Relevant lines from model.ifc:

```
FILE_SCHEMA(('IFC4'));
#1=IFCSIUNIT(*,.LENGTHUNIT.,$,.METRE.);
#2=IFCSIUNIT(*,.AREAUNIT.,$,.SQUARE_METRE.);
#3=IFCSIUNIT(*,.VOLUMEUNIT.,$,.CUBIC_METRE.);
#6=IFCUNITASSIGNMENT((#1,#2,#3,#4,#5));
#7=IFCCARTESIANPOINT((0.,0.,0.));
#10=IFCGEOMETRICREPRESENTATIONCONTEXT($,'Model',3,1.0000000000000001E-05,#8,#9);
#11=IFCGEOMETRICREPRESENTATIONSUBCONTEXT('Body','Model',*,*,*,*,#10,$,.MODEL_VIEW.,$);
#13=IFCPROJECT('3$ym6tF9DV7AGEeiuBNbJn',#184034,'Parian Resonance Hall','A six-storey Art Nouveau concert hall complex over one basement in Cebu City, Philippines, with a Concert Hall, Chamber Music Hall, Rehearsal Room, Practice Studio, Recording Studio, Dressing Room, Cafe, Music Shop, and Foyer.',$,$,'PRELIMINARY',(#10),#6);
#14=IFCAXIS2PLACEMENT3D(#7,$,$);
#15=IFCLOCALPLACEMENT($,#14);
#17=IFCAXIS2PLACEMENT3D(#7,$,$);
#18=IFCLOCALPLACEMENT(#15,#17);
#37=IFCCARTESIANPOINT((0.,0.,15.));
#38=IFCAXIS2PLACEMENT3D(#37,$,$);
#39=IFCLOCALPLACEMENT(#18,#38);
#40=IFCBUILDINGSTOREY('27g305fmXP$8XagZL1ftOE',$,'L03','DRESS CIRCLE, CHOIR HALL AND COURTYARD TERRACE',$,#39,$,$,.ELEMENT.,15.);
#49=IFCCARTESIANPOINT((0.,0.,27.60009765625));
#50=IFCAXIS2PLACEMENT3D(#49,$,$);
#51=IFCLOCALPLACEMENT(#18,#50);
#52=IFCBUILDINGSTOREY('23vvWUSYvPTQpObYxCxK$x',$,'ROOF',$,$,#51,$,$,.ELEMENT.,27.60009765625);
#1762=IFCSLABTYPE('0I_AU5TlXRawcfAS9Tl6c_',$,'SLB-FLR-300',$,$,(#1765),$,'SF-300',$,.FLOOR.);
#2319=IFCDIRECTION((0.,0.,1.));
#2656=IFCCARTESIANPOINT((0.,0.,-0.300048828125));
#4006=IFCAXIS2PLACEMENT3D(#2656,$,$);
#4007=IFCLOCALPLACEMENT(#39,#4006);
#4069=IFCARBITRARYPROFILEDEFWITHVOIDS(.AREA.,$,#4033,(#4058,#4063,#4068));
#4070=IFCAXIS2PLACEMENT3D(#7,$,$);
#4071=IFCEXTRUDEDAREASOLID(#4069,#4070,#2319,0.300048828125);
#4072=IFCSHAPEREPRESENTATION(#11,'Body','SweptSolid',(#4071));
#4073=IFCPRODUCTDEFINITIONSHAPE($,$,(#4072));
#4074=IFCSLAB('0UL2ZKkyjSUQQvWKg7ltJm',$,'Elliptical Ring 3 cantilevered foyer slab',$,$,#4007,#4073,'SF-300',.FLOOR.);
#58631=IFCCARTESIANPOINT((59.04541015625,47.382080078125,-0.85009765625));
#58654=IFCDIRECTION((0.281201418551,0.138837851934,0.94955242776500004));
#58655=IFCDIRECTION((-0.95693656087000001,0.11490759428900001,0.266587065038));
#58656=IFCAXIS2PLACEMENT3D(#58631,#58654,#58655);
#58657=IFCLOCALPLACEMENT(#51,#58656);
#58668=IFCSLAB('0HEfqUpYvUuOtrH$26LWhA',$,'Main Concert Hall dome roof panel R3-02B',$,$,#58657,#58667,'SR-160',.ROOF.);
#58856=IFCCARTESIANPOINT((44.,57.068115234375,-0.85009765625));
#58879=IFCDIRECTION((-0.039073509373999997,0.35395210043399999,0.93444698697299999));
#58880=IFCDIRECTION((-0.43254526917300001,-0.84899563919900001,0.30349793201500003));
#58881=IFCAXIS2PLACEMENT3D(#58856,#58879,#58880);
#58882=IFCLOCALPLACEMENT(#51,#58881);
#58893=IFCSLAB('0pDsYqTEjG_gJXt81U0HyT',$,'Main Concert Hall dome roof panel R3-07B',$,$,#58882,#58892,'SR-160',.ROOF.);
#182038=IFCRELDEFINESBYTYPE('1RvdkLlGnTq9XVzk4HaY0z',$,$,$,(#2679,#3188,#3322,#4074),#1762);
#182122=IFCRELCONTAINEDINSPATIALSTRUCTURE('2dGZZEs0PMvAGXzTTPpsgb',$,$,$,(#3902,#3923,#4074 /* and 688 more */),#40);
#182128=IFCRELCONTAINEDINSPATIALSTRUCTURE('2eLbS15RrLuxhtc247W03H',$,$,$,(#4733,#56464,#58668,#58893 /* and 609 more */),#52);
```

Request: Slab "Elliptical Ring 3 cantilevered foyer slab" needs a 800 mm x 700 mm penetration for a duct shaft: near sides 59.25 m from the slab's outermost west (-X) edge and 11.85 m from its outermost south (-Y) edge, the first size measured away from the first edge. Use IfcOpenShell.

```python
import numpy as np
import ifcopenshell
import ifcopenshell.api.feature
import ifcopenshell.api.geometry
import ifcopenshell.api.root
import ifcopenshell.geom
import ifcopenshell.util.placement
import ifcopenshell.util.representation
import ifcopenshell.util.shape
import ifcopenshell.util.unit

model = ifcopenshell.open("model.ifc")
unit_scale = ifcopenshell.util.unit.calculate_unit_scale(model)
settings = ifcopenshell.geom.settings()


def volume(element):
    """Net volume in cubic metres, openings subtracted."""
    shape = ifcopenshell.geom.create_shape(settings, element)
    return ifcopenshell.util.shape.get_volume(shape.geometry)


slab = model.by_id(4074)
before = volume(slab)

# Extent in the slab's own axes, in metres. The edges named are its -X and -Y sides.
slab_shape = ifcopenshell.geom.create_shape(settings, slab)
vertices = ifcopenshell.util.shape.get_vertices(slab_shape.geometry)
x_min, y_min, bottom = vertices.min(axis=0)
top = vertices[:, 2].max()

opening = ifcopenshell.api.root.create_entity(model, ifc_class="IfcOpeningElement", name="Duct shaft opening", predefined_type="OPENING")
context = ifcopenshell.util.representation.get_context(model, "Model", "Body", "MODEL_VIEW")
width, depth = 0.8, 0.7
outline = [(0.0, 0.0), (width, 0.0), (width, depth), (0.0, depth), (0.0, 0.0)]
# Overshoot both faces by 50 mm so the cut is clean.
shape = ifcopenshell.api.geometry.add_slab_representation(
    model, context=context, depth=top - bottom + 0.1, polyline=outline
)
ifcopenshell.api.geometry.assign_representation(model, product=opening, representation=shape)

matrix = ifcopenshell.util.placement.get_local_placement(slab.ObjectPlacement)
matrix[:, 3] = matrix @ np.append(np.array([x_min + 59.25, y_min + 11.85, bottom - 0.05]) / unit_scale, 1.0)
ifcopenshell.api.geometry.edit_object_placement(model, product=opening, matrix=matrix, is_si=False)
ifcopenshell.api.feature.add_feature(model, feature=opening, element=slab)

after = volume(slab)

print(f"slab volume {before:.3f} -> {after:.3f} m3")

model.write("model_edited.ifc")
```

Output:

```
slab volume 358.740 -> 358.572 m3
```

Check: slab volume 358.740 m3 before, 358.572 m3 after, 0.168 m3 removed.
